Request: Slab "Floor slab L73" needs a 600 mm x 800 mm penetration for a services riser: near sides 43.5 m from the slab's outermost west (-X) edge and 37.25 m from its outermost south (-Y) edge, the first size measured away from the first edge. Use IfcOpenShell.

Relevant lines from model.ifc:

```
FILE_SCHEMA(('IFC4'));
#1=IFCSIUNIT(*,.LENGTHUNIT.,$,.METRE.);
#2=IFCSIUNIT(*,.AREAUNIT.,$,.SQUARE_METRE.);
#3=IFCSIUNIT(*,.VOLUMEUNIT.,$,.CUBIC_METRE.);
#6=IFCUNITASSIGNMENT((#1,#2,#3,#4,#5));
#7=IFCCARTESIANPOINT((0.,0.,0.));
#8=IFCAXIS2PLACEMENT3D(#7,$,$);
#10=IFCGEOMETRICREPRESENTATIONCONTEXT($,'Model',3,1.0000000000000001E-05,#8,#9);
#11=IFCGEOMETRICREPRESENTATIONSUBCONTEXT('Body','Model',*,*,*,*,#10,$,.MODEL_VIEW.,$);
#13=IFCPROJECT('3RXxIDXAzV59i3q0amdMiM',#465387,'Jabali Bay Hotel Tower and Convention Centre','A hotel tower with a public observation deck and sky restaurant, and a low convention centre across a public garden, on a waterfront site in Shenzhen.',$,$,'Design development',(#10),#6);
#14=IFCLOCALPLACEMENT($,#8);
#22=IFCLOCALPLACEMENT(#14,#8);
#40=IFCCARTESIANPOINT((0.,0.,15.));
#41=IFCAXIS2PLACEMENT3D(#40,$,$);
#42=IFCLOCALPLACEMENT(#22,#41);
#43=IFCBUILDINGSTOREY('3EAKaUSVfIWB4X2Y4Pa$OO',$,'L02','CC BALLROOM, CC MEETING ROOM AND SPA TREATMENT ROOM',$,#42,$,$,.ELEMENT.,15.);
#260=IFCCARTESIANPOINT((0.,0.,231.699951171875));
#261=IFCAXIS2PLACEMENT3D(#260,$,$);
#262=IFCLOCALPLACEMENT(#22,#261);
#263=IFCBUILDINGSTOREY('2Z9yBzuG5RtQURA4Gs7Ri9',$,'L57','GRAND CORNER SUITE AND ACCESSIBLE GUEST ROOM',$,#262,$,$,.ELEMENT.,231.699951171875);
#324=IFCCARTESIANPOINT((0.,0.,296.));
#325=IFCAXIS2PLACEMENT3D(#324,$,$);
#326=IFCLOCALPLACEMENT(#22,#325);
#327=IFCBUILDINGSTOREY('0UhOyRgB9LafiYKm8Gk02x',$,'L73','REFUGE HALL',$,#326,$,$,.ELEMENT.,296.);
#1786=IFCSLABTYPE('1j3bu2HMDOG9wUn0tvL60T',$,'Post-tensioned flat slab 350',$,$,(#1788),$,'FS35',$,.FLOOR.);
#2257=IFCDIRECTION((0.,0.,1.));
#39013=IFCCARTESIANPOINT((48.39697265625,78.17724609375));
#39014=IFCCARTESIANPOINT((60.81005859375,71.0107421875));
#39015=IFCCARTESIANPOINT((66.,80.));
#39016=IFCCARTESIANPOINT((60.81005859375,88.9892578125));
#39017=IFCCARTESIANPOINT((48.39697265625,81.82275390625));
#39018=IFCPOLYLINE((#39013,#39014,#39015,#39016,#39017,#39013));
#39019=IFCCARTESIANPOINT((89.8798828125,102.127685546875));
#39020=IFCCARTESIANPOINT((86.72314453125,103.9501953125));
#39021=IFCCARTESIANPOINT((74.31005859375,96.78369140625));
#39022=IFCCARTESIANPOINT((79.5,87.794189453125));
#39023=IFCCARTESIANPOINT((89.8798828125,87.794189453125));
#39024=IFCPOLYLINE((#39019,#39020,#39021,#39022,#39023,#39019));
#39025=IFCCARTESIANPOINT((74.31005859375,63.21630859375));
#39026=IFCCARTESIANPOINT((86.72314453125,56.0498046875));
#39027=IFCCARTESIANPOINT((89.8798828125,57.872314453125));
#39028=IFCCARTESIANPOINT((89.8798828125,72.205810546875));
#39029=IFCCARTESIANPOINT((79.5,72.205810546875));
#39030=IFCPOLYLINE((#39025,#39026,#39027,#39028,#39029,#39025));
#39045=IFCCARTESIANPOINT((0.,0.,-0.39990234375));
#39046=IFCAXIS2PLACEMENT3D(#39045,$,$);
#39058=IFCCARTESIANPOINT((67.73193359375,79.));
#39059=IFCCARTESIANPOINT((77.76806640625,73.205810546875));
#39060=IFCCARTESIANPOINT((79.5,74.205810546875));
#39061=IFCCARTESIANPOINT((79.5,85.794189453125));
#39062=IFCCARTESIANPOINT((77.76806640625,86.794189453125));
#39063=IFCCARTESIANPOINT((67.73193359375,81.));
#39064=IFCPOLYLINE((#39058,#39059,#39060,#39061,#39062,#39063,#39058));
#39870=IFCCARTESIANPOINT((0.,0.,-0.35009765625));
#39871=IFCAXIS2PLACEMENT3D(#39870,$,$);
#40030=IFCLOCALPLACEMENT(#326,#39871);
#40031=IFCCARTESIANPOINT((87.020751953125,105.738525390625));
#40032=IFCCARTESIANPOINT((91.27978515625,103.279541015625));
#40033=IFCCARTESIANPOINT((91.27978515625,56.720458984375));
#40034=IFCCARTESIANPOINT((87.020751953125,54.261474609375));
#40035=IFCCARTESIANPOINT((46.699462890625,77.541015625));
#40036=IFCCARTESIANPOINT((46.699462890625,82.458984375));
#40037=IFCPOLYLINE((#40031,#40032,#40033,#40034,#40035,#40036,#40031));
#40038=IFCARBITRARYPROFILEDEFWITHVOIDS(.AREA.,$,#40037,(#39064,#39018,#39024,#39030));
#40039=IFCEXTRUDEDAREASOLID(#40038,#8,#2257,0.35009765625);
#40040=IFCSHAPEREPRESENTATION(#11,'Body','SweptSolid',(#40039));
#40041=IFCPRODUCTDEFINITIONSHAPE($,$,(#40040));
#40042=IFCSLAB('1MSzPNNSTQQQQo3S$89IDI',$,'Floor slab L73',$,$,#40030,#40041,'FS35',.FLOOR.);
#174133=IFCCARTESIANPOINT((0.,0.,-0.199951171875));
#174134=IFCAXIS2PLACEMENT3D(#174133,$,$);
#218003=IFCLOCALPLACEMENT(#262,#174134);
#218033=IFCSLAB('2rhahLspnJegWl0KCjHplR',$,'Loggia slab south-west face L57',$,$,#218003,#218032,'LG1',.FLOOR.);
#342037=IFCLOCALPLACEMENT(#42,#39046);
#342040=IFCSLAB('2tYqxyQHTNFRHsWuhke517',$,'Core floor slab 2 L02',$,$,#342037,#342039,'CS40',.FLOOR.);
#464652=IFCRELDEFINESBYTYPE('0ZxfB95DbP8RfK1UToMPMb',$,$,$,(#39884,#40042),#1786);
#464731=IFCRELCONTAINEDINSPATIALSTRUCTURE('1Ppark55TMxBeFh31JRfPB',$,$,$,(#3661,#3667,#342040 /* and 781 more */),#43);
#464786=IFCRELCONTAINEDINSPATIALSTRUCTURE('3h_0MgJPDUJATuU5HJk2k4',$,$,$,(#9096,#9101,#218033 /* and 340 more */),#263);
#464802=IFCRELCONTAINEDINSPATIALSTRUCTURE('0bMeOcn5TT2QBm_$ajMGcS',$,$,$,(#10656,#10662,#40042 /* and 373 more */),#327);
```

```python
import numpy as np
import ifcopenshell
import ifcopenshell.api.feature
import ifcopenshell.api.geometry
import ifcopenshell.api.root
import ifcopenshell.geom
import ifcopenshell.util.placement
import ifcopenshell.util.representation
import ifcopenshell.util.shape
import ifcopenshell.util.unit

model = ifcopenshell.open("model.ifc")
unit_scale = ifcopenshell.util.unit.calculate_unit_scale(model)
settings = ifcopenshell.geom.settings()


def volume(element):
    """Net volume in cubic metres, openings subtracted."""
    shape = ifcopenshell.geom.create_shape(settings, element)
    return ifcopenshell.util.shape.get_volume(shape.geometry)


slab = model.by_guid("1MSzPNNSTQQQQo3S$89IDI")
before = volume(slab)

# Extent in the slab's own axes, in metres. The edges named are its -X and -Y sides.
slab_shape = ifcopenshell.geom.create_shape(settings, slab)
vertices = ifcopenshell.util.shape.get_vertices(slab_shape.geometry)
x_min, y_min, bottom = vertices.min(axis=0)
top = vertices[:, 2].max()

opening = ifcopenshell.api.root.create_entity(model, ifc_class="IfcOpeningElement", name="Services riser opening", predefined_type="OPENING")
context = ifcopenshell.util.representation.get_context(model, "Model", "Body", "MODEL_VIEW")
width, depth = 0.6, 0.8
outline = [(0.0, 0.0), (width, 0.0), (width, depth), (0.0, depth), (0.0, 0.0)]
# Overshoot both faces by 50 mm so the cut is clean.
shape = ifcopenshell.api.geometry.add_slab_representation(
    model, context=context, depth=top - bottom + 0.1, polyline=outline
)
ifcopenshell.api.geometry.assign_representation(model, product=opening, representation=shape)

matrix = ifcopenshell.util.placement.get_local_placement(slab.ObjectPlacement)
matrix[:, 3] = matrix @ np.append(np.array([x_min + 43.5, y_min + 37.25, bottom - 0.05]) / unit_scale, 1.0)
ifcopenshell.api.geometry.edit_object_placement(model, product=opening, matrix=matrix, is_si=False)
ifcopenshell.api.feature.add_feature(model, feature=opening, element=slab)

after = volume(slab)

print(f"slab volume {before:.3f} -> {after:.3f} m3")

model.write("model-out.ifc")
```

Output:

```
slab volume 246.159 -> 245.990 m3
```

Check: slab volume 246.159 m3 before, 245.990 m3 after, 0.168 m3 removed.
